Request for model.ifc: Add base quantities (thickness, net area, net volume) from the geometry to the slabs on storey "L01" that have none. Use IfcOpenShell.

First a look at what the model holds.

```python
import ifcopenshell
import ifcopenshell.util.element
import ifcopenshell.util.unit

model = ifcopenshell.open("model.ifc")
print(model.schema)
for unit_type in ("LENGTHUNIT", "AREAUNIT", "VOLUMEUNIT"):
    print(unit_type, ifcopenshell.util.unit.calculate_unit_scale(model, unit_type))
storey = next(s for s in model.by_type("IfcBuildingStorey") if s.Name == "L01")
slabs = [e for e in ifcopenshell.util.element.get_decomposition(storey) if e.is_a("IfcSlab")]
for e in sorted(slabs, key=lambda e: e.id()):
    print(e.id(), e.is_a(), e.Name, list(ifcopenshell.util.element.get_psets(e, qtos_only=True)), sep=" | ")
```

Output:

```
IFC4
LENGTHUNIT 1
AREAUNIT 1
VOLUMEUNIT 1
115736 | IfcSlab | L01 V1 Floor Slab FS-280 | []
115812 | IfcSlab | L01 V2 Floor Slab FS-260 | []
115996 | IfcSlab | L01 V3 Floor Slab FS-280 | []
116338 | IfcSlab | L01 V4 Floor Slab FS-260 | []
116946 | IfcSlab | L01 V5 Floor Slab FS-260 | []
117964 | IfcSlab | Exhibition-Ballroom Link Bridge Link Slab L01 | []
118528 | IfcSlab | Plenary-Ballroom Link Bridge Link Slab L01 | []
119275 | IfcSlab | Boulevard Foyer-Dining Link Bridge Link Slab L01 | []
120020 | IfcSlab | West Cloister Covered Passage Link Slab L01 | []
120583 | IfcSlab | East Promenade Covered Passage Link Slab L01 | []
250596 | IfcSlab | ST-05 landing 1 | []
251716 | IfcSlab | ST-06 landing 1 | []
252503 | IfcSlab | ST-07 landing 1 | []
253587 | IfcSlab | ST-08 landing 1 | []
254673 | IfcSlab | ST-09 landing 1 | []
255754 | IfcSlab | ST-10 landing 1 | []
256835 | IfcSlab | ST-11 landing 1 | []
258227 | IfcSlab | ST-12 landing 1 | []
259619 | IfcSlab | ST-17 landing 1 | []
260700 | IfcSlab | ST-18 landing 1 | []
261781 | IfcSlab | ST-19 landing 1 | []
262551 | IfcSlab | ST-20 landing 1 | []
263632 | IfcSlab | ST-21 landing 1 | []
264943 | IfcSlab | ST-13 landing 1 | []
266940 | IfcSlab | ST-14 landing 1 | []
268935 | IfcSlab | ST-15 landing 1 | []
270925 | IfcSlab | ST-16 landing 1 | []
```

```python
import ifcopenshell
import ifcopenshell.api.pset
import ifcopenshell.geom
import ifcopenshell.util.element
import ifcopenshell.util.shape
import ifcopenshell.util.unit

model = ifcopenshell.open("model.ifc")
unit_scale = ifcopenshell.util.unit.calculate_unit_scale(model)
area_scale = ifcopenshell.util.unit.calculate_unit_scale(model, "AREAUNIT")
volume_scale = ifcopenshell.util.unit.calculate_unit_scale(model, "VOLUMEUNIT")
settings = ifcopenshell.geom.settings()

storey = next(s for s in model.by_type("IfcBuildingStorey") if s.Name == "L01")
slabs = [e for e in ifcopenshell.util.element.get_decomposition(storey) if e.is_a("IfcSlab")]

for e in sorted(slabs, key=lambda e: e.id()):
    if ifcopenshell.util.element.get_psets(e, qtos_only=True, should_inherit=False):
        continue
    # Geometry comes back in metres, in the element's own axes.
    shape = ifcopenshell.geom.create_shape(settings, e)
    values = {
        "Width": ifcopenshell.util.shape.get_z(shape.geometry) / unit_scale,
        "NetArea": ifcopenshell.util.shape.get_footprint_area(shape.geometry) / area_scale,
        "NetVolume": ifcopenshell.util.shape.get_volume(shape.geometry) / volume_scale,
    }
    qto = ifcopenshell.api.pset.add_qto(model, product=e, name="Qto_SlabBaseQuantities")
    ifcopenshell.api.pset.edit_qto(model, qto=qto, properties=values)
    print(e.id(), {k: round(v, 3) for k, v in values.items()})

model.write("model-out.ifc")
```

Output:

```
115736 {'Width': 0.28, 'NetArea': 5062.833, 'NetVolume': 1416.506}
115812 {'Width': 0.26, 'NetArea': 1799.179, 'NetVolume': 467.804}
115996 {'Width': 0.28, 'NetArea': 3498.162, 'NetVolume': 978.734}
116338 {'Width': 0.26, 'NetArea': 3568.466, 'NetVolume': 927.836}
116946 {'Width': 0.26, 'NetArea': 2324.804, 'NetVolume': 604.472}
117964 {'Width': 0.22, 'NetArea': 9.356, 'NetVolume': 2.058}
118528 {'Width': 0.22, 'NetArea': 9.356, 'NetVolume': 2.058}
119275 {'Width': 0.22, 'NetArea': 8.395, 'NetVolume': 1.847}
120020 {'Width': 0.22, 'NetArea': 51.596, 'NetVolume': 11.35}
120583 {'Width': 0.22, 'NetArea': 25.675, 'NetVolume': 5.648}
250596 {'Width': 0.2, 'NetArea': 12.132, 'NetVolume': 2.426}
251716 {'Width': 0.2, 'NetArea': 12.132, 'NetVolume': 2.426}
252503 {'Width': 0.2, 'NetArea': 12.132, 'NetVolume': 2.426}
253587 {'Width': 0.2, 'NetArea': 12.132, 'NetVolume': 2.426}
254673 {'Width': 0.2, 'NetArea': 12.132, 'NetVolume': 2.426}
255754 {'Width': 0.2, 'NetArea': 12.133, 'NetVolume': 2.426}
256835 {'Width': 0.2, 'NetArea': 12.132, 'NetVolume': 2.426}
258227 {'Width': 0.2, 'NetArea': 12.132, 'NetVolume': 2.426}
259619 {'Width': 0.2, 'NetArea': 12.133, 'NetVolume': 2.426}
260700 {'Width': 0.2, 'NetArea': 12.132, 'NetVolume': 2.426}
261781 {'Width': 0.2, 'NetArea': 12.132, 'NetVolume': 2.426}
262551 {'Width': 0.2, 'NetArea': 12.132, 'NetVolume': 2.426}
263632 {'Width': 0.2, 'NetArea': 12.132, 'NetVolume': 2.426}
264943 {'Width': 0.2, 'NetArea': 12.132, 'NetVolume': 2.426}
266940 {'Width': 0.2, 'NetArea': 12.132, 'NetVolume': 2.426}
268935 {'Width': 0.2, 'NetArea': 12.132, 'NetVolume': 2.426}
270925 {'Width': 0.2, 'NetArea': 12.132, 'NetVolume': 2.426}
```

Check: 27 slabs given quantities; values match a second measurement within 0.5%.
